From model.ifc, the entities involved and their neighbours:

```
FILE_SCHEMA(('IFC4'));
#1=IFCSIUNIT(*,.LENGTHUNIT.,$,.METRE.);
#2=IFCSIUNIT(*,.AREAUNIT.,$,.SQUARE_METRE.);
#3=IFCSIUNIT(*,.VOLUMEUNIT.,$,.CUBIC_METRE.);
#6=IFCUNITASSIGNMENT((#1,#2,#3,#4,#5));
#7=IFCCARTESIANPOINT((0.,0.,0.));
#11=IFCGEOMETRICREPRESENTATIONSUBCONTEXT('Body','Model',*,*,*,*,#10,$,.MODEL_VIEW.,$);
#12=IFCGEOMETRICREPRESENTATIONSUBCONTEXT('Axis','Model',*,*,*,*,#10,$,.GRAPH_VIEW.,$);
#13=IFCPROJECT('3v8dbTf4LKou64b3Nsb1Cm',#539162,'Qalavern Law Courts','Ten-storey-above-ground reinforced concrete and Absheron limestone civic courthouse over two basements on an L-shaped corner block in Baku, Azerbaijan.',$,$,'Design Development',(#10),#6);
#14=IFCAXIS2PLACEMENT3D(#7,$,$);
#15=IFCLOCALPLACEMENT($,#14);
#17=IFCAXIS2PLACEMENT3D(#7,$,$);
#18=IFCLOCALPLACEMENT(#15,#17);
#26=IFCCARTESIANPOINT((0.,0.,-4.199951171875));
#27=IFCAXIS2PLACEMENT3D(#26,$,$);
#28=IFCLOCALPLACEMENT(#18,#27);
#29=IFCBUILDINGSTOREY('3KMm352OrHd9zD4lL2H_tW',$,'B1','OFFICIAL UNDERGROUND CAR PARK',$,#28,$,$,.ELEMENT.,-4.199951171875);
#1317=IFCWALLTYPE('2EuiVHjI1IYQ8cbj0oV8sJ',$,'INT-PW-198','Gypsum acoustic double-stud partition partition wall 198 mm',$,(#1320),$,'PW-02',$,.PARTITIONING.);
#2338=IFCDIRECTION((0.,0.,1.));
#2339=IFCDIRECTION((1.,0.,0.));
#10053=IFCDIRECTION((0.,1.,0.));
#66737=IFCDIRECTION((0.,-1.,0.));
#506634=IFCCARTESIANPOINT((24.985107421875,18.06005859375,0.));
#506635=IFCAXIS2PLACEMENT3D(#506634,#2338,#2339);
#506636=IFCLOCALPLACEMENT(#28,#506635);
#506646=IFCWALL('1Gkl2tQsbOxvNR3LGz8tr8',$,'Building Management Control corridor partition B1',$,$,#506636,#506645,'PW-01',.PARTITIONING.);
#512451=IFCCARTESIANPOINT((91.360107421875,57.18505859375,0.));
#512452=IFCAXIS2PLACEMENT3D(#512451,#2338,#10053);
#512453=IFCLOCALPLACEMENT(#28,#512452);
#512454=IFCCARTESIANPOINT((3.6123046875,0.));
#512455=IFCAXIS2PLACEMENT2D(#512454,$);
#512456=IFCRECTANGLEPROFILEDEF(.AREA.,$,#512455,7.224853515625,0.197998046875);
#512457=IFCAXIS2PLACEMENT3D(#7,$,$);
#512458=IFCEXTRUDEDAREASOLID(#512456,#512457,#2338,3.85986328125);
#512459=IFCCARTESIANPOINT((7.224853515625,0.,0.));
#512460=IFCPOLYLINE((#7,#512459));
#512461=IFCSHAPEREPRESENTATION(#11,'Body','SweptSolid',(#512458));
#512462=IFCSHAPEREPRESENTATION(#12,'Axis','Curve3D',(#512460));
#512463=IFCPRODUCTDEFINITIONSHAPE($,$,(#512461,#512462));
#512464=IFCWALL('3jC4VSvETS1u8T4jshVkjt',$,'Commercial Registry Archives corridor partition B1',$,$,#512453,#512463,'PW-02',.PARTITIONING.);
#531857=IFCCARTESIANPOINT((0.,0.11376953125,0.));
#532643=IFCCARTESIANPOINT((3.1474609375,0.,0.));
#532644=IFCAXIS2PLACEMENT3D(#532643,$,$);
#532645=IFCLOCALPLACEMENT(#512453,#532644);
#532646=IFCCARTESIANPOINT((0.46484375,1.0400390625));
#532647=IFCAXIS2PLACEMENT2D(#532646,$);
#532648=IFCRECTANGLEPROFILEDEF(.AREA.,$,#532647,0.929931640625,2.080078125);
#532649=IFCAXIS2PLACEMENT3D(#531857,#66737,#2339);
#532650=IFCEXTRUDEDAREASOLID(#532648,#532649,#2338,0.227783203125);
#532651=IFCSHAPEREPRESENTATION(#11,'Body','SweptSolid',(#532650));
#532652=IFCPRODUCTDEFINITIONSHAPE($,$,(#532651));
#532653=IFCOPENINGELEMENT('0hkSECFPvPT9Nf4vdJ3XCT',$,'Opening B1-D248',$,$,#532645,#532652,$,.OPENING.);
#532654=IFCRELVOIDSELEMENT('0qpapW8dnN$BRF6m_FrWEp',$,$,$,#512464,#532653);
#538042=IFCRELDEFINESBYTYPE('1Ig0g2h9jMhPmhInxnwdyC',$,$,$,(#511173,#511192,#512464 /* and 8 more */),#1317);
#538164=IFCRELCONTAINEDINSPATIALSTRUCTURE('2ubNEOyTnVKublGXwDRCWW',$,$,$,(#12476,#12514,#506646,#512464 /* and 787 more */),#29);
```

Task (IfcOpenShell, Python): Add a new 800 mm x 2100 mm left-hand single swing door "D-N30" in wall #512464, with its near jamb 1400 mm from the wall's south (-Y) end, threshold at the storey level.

```python
import numpy as np
import ifcopenshell
import ifcopenshell.api.feature
import ifcopenshell.api.geometry
import ifcopenshell.api.root
import ifcopenshell.api.spatial
import ifcopenshell.geom
import ifcopenshell.util.element
import ifcopenshell.util.placement
import ifcopenshell.util.representation
import ifcopenshell.util.shape
import ifcopenshell.util.unit

model = ifcopenshell.open("model.ifc")
unit_scale = ifcopenshell.util.unit.calculate_unit_scale(model)
settings = ifcopenshell.geom.settings()


def volume(element):
    """Net volume in cubic metres, openings subtracted."""
    shape = ifcopenshell.geom.create_shape(settings, element)
    return ifcopenshell.util.shape.get_volume(shape.geometry)


wall = model.by_guid("3jC4VSvETS1u8T4jshVkjt")
storey = ifcopenshell.util.element.get_container(wall, ifc_class="IfcBuildingStorey")
context = ifcopenshell.util.representation.get_context(model, "Model", "Body", "MODEL_VIEW")
before = volume(wall)

width, height, from_end, sill = 0.8, 2.1, 1.4, 0.0  # metres

# The wall runs along its own X axis, and the end named is its -X end.
wall_shape = ifcopenshell.geom.create_shape(settings, wall)
x, y, z = ifcopenshell.util.shape.get_vertices(wall_shape.geometry).T
start = x.min() + from_end
face, thickness = float(y.min()), float(y.max() - y.min())
wall_matrix = ifcopenshell.util.placement.get_local_placement(wall.ObjectPlacement)
level = ifcopenshell.util.placement.get_local_placement(storey.ObjectPlacement)[2, 3]


def in_wall(x, y):
    """Placement at x, y metres in the wall's axes, at sill height."""
    matrix = wall_matrix.copy()
    matrix[:, 3] = wall_matrix @ np.array([x / unit_scale, y / unit_scale, 0.0, 1.0])
    matrix[2, 3] = level + sill / unit_scale
    return matrix


# Opening: a box that overshoots both wall faces by 50 mm.
opening = ifcopenshell.api.root.create_entity(model, ifc_class="IfcOpeningElement", predefined_type="OPENING")
box = ifcopenshell.api.geometry.add_wall_representation(
    model, context=context, length=width, height=height, thickness=thickness + 0.1
)
ifcopenshell.api.geometry.assign_representation(model, product=opening, representation=box)
ifcopenshell.api.geometry.edit_object_placement(model, product=opening, matrix=in_wall(start, face - 0.05), is_si=False)
ifcopenshell.api.feature.add_feature(model, feature=opening, element=wall)

door = ifcopenshell.api.root.create_entity(model, ifc_class="IfcDoor", name="D-N30", predefined_type="DOOR")
door.OverallWidth, door.OverallHeight = width / unit_scale, height / unit_scale
door.OperationType = "SINGLE_SWING_LEFT"
body = ifcopenshell.api.geometry.add_door_representation(
    model,
    context=context,
    overall_width=door.OverallWidth,
    overall_height=door.OverallHeight,
    operation_type="SINGLE_SWING_LEFT",
    lining_properties={"LiningDepth": thickness / unit_scale, "ThresholdDepth": thickness / unit_scale},
)
ifcopenshell.api.geometry.assign_representation(model, product=door, representation=body)
ifcopenshell.api.spatial.assign_container(model, products=[door], relating_structure=storey)
ifcopenshell.api.feature.add_filling(model, opening=opening, element=door)

# The lining spans the wall, so the door starts at the wall face.
ifcopenshell.api.geometry.edit_object_placement(model, product=door, matrix=in_wall(start, face), is_si=False)

after = volume(wall)

print(f"wall volume {before:.3f} -> {after:.3f} m3")

model.write("model-out.ifc")
```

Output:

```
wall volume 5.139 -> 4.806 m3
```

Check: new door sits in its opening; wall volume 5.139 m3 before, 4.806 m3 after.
